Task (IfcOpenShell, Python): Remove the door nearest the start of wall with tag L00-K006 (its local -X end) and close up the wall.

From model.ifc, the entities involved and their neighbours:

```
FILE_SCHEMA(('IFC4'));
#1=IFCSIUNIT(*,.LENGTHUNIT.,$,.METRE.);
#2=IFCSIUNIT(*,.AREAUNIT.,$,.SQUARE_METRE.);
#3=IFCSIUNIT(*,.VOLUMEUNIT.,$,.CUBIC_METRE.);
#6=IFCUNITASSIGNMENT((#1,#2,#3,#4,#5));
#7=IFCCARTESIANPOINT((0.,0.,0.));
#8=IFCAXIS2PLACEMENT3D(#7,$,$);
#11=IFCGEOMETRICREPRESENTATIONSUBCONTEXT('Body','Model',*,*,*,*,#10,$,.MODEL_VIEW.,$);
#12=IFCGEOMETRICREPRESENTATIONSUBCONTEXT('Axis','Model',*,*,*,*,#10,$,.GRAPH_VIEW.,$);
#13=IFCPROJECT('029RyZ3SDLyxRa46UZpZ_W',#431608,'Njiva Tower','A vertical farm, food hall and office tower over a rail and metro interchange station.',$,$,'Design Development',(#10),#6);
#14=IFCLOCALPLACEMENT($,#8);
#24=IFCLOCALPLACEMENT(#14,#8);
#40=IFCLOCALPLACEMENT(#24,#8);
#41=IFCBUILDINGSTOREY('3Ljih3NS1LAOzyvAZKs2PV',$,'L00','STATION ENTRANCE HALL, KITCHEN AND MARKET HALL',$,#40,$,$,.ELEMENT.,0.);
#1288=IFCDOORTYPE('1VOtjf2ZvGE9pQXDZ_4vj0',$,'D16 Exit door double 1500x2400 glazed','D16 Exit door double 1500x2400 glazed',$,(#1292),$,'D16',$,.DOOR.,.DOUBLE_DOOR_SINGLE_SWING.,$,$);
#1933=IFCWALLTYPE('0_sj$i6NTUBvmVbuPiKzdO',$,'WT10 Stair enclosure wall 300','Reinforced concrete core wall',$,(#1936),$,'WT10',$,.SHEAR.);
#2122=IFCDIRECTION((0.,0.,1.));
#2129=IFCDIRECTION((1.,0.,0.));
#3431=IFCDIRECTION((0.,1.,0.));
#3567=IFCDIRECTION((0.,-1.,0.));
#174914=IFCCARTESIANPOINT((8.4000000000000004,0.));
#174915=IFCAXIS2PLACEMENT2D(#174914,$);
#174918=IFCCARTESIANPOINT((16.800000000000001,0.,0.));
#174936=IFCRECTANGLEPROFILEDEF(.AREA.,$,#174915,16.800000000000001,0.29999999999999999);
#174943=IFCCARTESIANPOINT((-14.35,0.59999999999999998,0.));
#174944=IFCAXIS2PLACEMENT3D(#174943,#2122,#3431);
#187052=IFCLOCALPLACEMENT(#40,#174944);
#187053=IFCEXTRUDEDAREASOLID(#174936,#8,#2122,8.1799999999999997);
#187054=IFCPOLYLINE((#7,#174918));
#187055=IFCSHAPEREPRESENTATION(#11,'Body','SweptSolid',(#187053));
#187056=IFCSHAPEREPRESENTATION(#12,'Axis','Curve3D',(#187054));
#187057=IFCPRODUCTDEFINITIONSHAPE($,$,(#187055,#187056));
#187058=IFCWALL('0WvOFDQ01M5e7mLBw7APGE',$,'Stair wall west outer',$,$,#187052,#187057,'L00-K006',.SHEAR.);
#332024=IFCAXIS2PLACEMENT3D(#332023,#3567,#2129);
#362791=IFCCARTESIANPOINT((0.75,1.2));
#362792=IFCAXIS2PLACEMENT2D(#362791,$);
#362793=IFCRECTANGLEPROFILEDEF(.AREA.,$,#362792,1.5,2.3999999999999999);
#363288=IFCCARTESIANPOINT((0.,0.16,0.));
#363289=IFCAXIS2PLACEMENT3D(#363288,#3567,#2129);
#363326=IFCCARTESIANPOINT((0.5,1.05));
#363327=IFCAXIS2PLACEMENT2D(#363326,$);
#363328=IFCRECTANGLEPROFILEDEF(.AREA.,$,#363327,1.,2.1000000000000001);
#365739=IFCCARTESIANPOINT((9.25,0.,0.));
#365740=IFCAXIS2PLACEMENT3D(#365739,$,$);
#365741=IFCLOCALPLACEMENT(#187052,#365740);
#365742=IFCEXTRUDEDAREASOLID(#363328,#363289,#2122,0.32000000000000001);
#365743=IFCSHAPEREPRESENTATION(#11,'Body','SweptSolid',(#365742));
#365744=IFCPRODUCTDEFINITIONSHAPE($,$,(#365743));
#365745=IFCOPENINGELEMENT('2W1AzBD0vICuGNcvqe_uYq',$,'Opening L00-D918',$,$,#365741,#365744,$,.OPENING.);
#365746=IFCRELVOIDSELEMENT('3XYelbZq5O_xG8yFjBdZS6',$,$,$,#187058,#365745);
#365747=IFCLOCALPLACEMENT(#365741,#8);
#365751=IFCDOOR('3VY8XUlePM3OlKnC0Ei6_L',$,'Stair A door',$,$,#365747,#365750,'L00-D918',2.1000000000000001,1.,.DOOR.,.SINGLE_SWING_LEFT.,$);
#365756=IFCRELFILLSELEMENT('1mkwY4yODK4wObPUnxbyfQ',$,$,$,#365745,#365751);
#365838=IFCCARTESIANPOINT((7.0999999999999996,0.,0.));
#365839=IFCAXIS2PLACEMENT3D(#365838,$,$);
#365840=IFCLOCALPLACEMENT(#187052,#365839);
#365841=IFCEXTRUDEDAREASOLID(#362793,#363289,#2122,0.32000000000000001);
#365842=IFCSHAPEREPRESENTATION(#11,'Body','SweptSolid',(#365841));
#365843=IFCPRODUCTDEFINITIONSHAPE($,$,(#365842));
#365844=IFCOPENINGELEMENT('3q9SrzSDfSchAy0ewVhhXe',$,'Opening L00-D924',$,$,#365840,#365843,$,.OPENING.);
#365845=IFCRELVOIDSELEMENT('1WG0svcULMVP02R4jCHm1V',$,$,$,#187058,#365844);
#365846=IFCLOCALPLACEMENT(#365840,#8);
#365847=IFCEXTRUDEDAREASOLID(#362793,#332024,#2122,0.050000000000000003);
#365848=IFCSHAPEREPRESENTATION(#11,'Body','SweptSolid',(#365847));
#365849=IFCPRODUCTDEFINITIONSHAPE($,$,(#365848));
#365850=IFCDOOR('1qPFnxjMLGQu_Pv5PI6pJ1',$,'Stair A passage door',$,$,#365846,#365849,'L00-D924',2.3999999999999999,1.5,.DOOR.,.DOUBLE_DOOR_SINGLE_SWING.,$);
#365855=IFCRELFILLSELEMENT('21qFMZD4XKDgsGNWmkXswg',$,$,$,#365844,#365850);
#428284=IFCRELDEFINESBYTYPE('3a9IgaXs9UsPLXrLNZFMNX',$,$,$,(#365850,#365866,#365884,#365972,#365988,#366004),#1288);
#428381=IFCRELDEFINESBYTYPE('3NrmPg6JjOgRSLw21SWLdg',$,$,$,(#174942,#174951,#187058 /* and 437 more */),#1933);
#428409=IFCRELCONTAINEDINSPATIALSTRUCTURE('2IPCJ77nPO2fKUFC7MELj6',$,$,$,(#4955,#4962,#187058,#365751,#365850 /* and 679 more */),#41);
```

```python
import ifcopenshell
import ifcopenshell.api.feature
import ifcopenshell.api.root
import ifcopenshell.geom
import ifcopenshell.util.shape

model = ifcopenshell.open("model.ifc")
settings = ifcopenshell.geom.settings()


def volume(element):
    """Net volume in cubic metres, openings subtracted."""
    shape = ifcopenshell.geom.create_shape(settings, element)
    return ifcopenshell.util.shape.get_volume(shape.geometry)


door = model.by_guid("1qPFnxjMLGQu_Pv5PI6pJ1")
opening = door.FillsVoids[0].RelatingOpeningElement
wall = opening.VoidsElements[0].RelatingBuildingElement
before = volume(wall)

ifcopenshell.api.root.remove_product(model, product=door)
ifcopenshell.api.feature.remove_feature(model, feature=opening)

after = volume(wall)

print(f"wall volume {before:.3f} -> {after:.3f} m3")

model.write("model_edited.ifc")
```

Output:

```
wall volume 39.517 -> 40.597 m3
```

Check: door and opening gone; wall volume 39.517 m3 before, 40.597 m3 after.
